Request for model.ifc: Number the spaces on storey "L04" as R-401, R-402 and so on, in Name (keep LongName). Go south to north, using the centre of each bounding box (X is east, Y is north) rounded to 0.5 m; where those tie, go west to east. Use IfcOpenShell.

First a look at what the model holds.

```python
import ifcopenshell
import ifcopenshell.util.element
import ifcopenshell.util.placement

model = ifcopenshell.open("model.ifc")
print(model.schema)
storey = next(s for s in model.by_type("IfcBuildingStorey") if s.Name == "L04")
spaces = [e for e in ifcopenshell.util.element.get_decomposition(storey) if e.is_a("IfcSpace")]
for e in sorted(spaces, key=lambda e: e.id()):
    origin = ifcopenshell.util.placement.get_local_placement(e.ObjectPlacement)[:3, 3]
    print(e.id(), e.Name, e.LongName, origin.round(2) + 0.0, sep=" | ")
```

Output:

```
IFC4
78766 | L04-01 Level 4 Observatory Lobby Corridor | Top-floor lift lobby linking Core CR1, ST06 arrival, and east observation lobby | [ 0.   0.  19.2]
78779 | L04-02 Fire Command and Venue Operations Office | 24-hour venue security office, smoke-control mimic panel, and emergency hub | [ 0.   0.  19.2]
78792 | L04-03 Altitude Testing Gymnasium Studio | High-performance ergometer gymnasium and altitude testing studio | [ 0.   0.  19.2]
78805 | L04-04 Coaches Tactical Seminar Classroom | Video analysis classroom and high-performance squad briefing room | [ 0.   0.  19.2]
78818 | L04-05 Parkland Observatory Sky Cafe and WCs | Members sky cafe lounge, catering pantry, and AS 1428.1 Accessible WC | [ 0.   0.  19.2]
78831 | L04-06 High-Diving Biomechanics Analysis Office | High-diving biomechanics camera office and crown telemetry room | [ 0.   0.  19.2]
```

```python
import ifcopenshell
import ifcopenshell.geom
import ifcopenshell.util.element
import ifcopenshell.util.shape

model = ifcopenshell.open("model.ifc")
settings = ifcopenshell.geom.settings()
settings.set("use-world-coords", True)


def centre(element):
    shape = ifcopenshell.geom.create_shape(settings, element)
    return ifcopenshell.util.shape.get_bbox_centroid(shape.geometry)


storey = next(s for s in model.by_type("IfcBuildingStorey") if s.Name == "L04")
spaces = [e for e in ifcopenshell.util.element.get_decomposition(storey) if e.is_a("IfcSpace")]

# Insertion points can sit at a corner or the storey origin, so sort by the geometry (in metres).
centres = {e: centre(e) for e in spaces}
spaces.sort(key=lambda e: (round(centres[e][1] / 0.5), centres[e][0]))

for i, e in enumerate(spaces, start=1):
    number = f"R-4{i:02d}"
    e.Name = number
    print(e.id(), number)

model.write("model_v2.ifc")
```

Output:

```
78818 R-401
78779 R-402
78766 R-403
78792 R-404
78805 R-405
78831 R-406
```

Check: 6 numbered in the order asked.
